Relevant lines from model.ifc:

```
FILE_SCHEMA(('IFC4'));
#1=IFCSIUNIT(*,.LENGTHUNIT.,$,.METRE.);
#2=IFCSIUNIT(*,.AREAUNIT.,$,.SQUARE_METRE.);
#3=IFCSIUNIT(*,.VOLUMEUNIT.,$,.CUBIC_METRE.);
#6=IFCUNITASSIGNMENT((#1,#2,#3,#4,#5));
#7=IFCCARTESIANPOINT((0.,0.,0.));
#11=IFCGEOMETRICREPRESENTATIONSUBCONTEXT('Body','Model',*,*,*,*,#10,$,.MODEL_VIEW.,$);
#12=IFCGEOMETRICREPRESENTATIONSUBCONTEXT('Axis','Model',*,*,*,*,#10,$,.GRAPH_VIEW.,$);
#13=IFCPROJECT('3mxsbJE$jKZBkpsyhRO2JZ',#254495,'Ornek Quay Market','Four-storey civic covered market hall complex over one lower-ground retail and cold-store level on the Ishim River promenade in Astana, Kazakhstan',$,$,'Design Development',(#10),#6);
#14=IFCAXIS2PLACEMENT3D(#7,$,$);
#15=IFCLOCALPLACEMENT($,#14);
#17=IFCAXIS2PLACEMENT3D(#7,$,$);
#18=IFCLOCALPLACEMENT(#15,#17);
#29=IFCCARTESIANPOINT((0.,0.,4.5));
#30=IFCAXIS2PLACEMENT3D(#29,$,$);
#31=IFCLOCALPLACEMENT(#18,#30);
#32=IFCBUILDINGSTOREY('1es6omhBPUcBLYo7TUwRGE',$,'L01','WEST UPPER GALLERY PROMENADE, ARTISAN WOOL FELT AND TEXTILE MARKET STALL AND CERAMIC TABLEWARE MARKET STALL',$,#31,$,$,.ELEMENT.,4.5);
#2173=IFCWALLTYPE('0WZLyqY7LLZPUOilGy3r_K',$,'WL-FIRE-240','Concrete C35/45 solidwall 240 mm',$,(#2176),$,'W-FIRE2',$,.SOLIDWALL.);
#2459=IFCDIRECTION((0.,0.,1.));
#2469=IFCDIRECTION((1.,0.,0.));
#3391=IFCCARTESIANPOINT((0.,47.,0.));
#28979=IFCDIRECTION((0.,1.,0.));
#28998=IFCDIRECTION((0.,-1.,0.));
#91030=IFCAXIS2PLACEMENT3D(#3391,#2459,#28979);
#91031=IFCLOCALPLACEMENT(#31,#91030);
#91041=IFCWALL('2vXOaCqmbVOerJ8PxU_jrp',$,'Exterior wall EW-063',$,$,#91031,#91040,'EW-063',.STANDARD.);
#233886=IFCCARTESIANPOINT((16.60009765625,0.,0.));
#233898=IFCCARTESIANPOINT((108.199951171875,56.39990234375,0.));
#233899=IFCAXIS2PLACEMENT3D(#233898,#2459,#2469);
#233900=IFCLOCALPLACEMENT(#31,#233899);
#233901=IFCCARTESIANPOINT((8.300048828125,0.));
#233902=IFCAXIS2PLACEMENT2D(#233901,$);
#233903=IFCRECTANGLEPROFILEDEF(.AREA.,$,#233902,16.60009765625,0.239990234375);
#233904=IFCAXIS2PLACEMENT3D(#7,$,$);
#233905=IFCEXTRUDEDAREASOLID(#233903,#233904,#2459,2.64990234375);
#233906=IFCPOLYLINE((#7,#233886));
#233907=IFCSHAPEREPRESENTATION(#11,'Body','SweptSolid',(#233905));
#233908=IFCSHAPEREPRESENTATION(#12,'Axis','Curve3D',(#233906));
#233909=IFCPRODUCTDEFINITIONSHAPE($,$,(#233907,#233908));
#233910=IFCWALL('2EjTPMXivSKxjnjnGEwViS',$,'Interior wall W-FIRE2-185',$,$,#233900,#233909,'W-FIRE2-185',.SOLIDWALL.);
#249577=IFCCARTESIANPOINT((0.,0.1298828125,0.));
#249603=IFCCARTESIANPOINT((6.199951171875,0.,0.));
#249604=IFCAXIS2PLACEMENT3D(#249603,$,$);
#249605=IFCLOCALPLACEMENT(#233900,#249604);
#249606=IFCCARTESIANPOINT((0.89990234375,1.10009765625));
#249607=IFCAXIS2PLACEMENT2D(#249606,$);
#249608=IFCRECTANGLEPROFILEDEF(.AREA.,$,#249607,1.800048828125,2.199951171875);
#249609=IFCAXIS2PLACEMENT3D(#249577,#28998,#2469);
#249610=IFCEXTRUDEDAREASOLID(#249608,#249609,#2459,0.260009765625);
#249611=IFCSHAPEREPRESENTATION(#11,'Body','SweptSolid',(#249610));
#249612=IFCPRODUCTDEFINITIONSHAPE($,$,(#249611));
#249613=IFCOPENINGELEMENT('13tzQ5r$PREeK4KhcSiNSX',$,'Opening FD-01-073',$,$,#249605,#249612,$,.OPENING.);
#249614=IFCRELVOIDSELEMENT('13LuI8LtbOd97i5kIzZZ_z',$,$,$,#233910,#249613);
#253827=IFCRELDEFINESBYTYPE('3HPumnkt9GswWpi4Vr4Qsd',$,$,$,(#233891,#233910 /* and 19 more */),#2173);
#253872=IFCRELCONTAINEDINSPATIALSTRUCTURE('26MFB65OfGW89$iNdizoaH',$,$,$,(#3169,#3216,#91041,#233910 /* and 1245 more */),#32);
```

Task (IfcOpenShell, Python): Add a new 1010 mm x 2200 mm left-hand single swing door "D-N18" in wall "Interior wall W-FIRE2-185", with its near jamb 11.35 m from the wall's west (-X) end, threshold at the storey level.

```python
import numpy as np
import ifcopenshell
import ifcopenshell.api.feature
import ifcopenshell.api.geometry
import ifcopenshell.api.root
import ifcopenshell.api.spatial
import ifcopenshell.geom
import ifcopenshell.util.element
import ifcopenshell.util.placement
import ifcopenshell.util.representation
import ifcopenshell.util.shape
import ifcopenshell.util.unit

model = ifcopenshell.open("model.ifc")
unit_scale = ifcopenshell.util.unit.calculate_unit_scale(model)
settings = ifcopenshell.geom.settings()


def volume(element):
    """Net volume in cubic metres, openings subtracted."""
    shape = ifcopenshell.geom.create_shape(settings, element)
    return ifcopenshell.util.shape.get_volume(shape.geometry)


wall = model.by_guid("2EjTPMXivSKxjnjnGEwViS")
storey = ifcopenshell.util.element.get_container(wall, ifc_class="IfcBuildingStorey")
context = ifcopenshell.util.representation.get_context(model, "Model", "Body", "MODEL_VIEW")
before = volume(wall)

width, height, from_end, sill = 1.01, 2.2, 11.35, 0.0  # metres

# The wall runs along its own X axis, and the end named is its -X end.
wall_shape = ifcopenshell.geom.create_shape(settings, wall)
x, y, z = ifcopenshell.util.shape.get_vertices(wall_shape.geometry).T
start = x.min() + from_end
face, thickness = float(y.min()), float(y.max() - y.min())
wall_matrix = ifcopenshell.util.placement.get_local_placement(wall.ObjectPlacement)
level = ifcopenshell.util.placement.get_local_placement(storey.ObjectPlacement)[2, 3]


def in_wall(x, y):
    """Placement at x, y metres in the wall's axes, at sill height."""
    matrix = wall_matrix.copy()
    matrix[:, 3] = wall_matrix @ np.array([x / unit_scale, y / unit_scale, 0.0, 1.0])
    matrix[2, 3] = level + sill / unit_scale
    return matrix


# Opening: a box that overshoots both wall faces by 50 mm.
opening = ifcopenshell.api.root.create_entity(model, ifc_class="IfcOpeningElement", predefined_type="OPENING")
box = ifcopenshell.api.geometry.add_wall_representation(
    model, context=context, length=width, height=height, thickness=thickness + 0.1
)
ifcopenshell.api.geometry.assign_representation(model, product=opening, representation=box)
ifcopenshell.api.geometry.edit_object_placement(model, product=opening, matrix=in_wall(start, face - 0.05), is_si=False)
ifcopenshell.api.feature.add_feature(model, feature=opening, element=wall)

door = ifcopenshell.api.root.create_entity(model, ifc_class="IfcDoor", name="D-N18", predefined_type="DOOR")
door.OverallWidth, door.OverallHeight = width / unit_scale, height / unit_scale
door.OperationType = "SINGLE_SWING_LEFT"
body = ifcopenshell.api.geometry.add_door_representation(
    model,
    context=context,
    overall_width=door.OverallWidth,
    overall_height=door.OverallHeight,
    operation_type="SINGLE_SWING_LEFT",
    lining_properties={"LiningDepth": thickness / unit_scale, "ThresholdDepth": thickness / unit_scale},
)
ifcopenshell.api.geometry.assign_representation(model, product=door, representation=body)
ifcopenshell.api.spatial.assign_container(model, products=[door], relating_structure=storey)
ifcopenshell.api.feature.add_filling(model, opening=opening, element=door)

# The lining spans the wall, so the door starts at the wall face.
ifcopenshell.api.geometry.edit_object_placement(model, product=door, matrix=in_wall(start, face), is_si=False)

after = volume(wall)

print(f"wall volume {before:.3f} -> {after:.3f} m3")

model.write("model_rev.ifc")
```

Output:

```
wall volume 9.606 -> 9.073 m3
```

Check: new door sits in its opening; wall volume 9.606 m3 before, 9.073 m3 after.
